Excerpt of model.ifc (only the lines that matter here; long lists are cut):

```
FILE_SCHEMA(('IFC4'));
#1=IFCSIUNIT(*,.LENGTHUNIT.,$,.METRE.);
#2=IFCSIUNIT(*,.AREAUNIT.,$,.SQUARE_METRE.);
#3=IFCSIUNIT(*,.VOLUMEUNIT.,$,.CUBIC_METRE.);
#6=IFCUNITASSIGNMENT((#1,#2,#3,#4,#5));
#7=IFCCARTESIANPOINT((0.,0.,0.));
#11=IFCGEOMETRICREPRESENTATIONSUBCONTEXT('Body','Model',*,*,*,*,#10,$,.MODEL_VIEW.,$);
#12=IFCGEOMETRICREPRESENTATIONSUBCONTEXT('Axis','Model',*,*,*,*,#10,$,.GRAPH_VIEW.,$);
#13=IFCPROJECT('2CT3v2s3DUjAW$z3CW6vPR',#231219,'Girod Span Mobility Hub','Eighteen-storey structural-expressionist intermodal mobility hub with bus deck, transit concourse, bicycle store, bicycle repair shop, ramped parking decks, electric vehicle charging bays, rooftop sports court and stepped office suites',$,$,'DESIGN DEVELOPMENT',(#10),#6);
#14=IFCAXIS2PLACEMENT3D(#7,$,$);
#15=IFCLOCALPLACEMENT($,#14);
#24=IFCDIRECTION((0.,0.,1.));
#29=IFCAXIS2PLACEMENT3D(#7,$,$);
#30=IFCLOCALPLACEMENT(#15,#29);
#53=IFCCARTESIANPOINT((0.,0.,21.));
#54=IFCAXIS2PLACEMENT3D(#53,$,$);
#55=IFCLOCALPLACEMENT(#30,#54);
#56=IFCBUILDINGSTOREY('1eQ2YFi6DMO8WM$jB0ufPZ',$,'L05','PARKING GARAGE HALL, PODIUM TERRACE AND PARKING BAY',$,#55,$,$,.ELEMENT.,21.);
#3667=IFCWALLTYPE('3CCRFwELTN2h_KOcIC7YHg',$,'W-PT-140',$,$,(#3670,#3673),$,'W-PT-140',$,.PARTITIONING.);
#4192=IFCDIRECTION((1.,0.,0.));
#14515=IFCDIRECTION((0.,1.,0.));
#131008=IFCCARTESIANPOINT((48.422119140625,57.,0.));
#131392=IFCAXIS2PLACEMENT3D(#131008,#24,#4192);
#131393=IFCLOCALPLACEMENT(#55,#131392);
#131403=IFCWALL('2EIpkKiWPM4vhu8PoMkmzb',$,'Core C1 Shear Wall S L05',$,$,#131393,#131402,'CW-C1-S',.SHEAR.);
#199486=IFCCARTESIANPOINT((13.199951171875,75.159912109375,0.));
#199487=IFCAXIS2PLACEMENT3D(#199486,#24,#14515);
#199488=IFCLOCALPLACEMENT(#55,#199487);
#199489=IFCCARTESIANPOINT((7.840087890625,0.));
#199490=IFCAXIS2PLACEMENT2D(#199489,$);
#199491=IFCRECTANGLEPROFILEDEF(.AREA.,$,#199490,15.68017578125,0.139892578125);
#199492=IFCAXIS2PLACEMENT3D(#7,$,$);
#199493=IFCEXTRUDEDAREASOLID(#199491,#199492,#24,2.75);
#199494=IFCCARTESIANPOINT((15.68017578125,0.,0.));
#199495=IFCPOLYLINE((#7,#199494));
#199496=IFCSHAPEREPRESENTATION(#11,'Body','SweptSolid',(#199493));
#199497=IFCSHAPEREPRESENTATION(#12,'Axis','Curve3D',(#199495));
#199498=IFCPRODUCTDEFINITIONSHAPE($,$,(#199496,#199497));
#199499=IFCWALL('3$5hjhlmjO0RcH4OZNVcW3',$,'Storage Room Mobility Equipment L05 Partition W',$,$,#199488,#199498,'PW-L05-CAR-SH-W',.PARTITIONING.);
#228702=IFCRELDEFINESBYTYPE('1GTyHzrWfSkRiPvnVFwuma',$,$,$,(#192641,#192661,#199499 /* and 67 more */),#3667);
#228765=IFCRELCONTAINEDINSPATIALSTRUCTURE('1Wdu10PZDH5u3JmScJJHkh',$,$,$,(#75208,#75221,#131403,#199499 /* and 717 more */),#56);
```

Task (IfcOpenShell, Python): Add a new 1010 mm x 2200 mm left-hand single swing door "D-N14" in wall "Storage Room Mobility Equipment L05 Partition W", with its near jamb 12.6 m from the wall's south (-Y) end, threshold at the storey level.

```python
import numpy as np
import ifcopenshell
import ifcopenshell.api.feature
import ifcopenshell.api.geometry
import ifcopenshell.api.root
import ifcopenshell.api.spatial
import ifcopenshell.geom
import ifcopenshell.util.element
import ifcopenshell.util.placement
import ifcopenshell.util.representation
import ifcopenshell.util.shape
import ifcopenshell.util.unit

model = ifcopenshell.open("model.ifc")
unit_scale = ifcopenshell.util.unit.calculate_unit_scale(model)
settings = ifcopenshell.geom.settings()


def volume(element):
    """Net volume in cubic metres, openings subtracted."""
    shape = ifcopenshell.geom.create_shape(settings, element)
    return ifcopenshell.util.shape.get_volume(shape.geometry)


wall = model.by_guid("3$5hjhlmjO0RcH4OZNVcW3")
storey = ifcopenshell.util.element.get_container(wall, ifc_class="IfcBuildingStorey")
context = ifcopenshell.util.representation.get_context(model, "Model", "Body", "MODEL_VIEW")
before = volume(wall)

width, height, from_end, sill = 1.01, 2.2, 12.6, 0.0  # metres

# The wall runs along its own X axis, and the end named is its -X end.
wall_shape = ifcopenshell.geom.create_shape(settings, wall)
x, y, z = ifcopenshell.util.shape.get_vertices(wall_shape.geometry).T
start = x.min() + from_end
face, thickness = float(y.min()), float(y.max() - y.min())
wall_matrix = ifcopenshell.util.placement.get_local_placement(wall.ObjectPlacement)
level = ifcopenshell.util.placement.get_local_placement(storey.ObjectPlacement)[2, 3]


def in_wall(x, y):
    """Placement at x, y metres in the wall's axes, at sill height."""
    matrix = wall_matrix.copy()
    matrix[:, 3] = wall_matrix @ np.array([x / unit_scale, y / unit_scale, 0.0, 1.0])
    matrix[2, 3] = level + sill / unit_scale
    return matrix


# Opening: a box that overshoots both wall faces by 50 mm.
opening = ifcopenshell.api.root.create_entity(model, ifc_class="IfcOpeningElement", predefined_type="OPENING")
box = ifcopenshell.api.geometry.add_wall_representation(
    model, context=context, length=width, height=height, thickness=thickness + 0.1
)
ifcopenshell.api.geometry.assign_representation(model, product=opening, representation=box)
ifcopenshell.api.geometry.edit_object_placement(model, product=opening, matrix=in_wall(start, face - 0.05), is_si=False)
ifcopenshell.api.feature.add_feature(model, feature=opening, element=wall)

door = ifcopenshell.api.root.create_entity(model, ifc_class="IfcDoor", name="D-N14", predefined_type="DOOR")
door.OverallWidth, door.OverallHeight = width / unit_scale, height / unit_scale
door.OperationType = "SINGLE_SWING_LEFT"
body = ifcopenshell.api.geometry.add_door_representation(
    model,
    context=context,
    overall_width=door.OverallWidth,
    overall_height=door.OverallHeight,
    operation_type="SINGLE_SWING_LEFT",
    lining_properties={"LiningDepth": thickness / unit_scale, "ThresholdDepth": thickness / unit_scale},
)
ifcopenshell.api.geometry.assign_representation(model, product=door, representation=body)
ifcopenshell.api.spatial.assign_container(model, products=[door], relating_structure=storey)
ifcopenshell.api.feature.add_filling(model, opening=opening, element=door)

# The lining spans the wall, so the door starts at the wall face.
ifcopenshell.api.geometry.edit_object_placement(model, product=door, matrix=in_wall(start, face), is_si=False)

after = volume(wall)

print(f"wall volume {before:.3f} -> {after:.3f} m3")

model.write("model_updated.ifc")
```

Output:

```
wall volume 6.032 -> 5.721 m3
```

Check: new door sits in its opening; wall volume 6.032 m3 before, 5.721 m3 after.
